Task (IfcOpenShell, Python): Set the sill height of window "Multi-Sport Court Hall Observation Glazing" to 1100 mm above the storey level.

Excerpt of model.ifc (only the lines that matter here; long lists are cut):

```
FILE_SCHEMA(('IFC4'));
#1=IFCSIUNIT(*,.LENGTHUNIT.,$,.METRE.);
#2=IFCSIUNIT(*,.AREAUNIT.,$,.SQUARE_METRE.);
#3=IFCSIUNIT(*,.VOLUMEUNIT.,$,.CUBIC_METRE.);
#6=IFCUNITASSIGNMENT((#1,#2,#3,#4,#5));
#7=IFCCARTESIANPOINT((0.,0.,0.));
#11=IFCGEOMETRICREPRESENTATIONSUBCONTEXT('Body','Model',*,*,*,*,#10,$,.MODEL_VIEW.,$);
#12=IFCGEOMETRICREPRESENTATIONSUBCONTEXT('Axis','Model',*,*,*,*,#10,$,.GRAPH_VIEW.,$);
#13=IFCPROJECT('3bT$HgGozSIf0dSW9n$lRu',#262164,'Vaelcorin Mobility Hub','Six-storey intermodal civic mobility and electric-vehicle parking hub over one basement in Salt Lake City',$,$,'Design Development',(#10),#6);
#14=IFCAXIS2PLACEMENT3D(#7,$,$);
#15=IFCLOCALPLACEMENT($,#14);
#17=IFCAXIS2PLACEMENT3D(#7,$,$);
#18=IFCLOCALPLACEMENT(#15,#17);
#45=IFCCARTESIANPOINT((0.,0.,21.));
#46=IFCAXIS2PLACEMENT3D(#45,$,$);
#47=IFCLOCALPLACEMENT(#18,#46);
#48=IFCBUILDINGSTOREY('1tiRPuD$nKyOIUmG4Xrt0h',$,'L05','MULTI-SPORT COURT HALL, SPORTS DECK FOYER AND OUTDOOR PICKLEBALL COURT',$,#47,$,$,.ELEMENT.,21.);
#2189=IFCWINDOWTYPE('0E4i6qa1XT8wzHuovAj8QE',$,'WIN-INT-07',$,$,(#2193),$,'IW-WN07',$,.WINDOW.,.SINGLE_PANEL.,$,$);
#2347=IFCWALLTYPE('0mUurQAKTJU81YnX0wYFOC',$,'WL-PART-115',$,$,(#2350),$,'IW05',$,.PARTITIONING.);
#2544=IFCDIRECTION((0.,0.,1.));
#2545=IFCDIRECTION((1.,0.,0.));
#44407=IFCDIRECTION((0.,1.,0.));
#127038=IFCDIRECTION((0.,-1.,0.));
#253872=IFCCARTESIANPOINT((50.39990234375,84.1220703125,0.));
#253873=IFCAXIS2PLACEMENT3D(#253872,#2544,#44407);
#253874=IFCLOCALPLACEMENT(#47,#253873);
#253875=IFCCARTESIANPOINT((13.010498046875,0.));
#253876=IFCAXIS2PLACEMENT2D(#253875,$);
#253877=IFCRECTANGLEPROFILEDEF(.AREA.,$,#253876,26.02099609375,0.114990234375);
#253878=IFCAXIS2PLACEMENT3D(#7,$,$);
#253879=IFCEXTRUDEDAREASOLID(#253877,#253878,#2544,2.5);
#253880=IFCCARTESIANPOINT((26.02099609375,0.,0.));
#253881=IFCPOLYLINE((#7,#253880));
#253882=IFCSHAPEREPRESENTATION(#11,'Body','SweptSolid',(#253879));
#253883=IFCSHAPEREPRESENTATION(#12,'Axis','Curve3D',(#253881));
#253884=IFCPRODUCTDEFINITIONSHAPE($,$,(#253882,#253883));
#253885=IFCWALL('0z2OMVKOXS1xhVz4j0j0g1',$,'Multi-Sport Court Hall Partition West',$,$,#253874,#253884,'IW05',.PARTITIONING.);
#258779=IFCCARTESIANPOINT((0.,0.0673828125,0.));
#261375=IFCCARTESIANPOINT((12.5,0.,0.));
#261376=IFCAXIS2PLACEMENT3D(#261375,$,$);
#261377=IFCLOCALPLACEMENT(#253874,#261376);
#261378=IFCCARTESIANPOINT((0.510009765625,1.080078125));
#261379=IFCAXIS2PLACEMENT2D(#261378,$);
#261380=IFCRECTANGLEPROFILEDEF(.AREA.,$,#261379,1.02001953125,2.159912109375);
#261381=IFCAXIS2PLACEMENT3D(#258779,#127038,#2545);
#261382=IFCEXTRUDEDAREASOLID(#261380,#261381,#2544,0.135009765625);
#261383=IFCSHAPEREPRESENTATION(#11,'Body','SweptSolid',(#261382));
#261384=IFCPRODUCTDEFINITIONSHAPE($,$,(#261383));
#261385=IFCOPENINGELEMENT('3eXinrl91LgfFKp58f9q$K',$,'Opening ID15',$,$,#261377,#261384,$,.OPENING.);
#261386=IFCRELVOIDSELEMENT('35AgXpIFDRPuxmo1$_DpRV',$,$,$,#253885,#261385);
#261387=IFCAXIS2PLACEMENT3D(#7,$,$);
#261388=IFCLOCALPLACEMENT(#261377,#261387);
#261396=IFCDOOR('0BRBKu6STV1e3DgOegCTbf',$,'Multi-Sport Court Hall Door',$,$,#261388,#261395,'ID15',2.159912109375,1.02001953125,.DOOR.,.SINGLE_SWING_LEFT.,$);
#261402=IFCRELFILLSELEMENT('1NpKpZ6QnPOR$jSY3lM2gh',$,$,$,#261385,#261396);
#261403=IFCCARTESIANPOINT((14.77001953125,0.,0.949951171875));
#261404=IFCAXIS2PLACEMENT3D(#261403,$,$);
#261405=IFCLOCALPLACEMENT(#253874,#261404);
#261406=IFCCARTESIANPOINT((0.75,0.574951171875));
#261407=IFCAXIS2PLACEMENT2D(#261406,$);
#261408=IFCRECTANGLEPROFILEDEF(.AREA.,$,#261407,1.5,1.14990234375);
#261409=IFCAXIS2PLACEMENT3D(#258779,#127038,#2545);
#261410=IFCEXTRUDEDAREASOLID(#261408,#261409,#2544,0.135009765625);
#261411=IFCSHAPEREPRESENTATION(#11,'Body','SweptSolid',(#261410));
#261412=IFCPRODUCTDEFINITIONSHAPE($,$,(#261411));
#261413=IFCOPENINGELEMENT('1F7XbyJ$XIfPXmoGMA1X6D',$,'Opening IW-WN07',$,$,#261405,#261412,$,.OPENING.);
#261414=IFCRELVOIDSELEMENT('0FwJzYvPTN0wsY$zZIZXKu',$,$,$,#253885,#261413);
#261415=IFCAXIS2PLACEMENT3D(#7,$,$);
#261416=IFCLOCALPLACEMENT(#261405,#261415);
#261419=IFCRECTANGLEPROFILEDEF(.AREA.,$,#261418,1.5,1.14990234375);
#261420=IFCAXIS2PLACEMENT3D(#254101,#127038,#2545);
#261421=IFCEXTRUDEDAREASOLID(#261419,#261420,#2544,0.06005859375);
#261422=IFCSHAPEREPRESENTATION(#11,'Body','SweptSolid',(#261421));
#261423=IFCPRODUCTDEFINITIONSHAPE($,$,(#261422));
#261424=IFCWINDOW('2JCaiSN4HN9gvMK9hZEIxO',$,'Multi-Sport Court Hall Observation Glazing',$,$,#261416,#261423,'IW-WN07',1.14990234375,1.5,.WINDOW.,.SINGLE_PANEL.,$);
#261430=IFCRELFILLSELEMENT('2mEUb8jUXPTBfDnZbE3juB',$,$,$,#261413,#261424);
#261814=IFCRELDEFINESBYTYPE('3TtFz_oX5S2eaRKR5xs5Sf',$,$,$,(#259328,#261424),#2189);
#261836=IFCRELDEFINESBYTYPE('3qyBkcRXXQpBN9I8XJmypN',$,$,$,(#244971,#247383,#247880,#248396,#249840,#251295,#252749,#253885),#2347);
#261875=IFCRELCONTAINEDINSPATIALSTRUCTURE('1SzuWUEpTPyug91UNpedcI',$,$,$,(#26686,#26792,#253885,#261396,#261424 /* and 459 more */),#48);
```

```python
import numpy as np
import ifcopenshell
import ifcopenshell.api.geometry
import ifcopenshell.geom
import ifcopenshell.util.element
import ifcopenshell.util.placement
import ifcopenshell.util.shape
import ifcopenshell.util.unit

model = ifcopenshell.open("model.ifc")
unit_scale = ifcopenshell.util.unit.calculate_unit_scale(model)

window = model.by_guid("2JCaiSN4HN9gvMK9hZEIxO")
opening = window.FillsVoids[0].RelatingOpeningElement
storey = ifcopenshell.util.element.get_container(window, ifc_class="IfcBuildingStorey")
level = ifcopenshell.util.placement.get_local_placement(storey.ObjectPlacement)[2, 3]

# The opening's origin need not be at the sill, so measure its lowest point.
shape = ifcopenshell.geom.create_shape(ifcopenshell.geom.settings(), opening)
bottom = ifcopenshell.util.shape.get_shape_bottom_elevation(shape, shape.geometry) / unit_scale
dz = level + 1.1 / unit_scale - bottom

shift = np.array([0.0, 0.0, dz])
# The window is placed relative to its opening, so it follows when the opening moves.
matrix = ifcopenshell.util.placement.get_local_placement(opening.ObjectPlacement)
matrix[:3, 3] += shift
ifcopenshell.api.geometry.edit_object_placement(
    model, product=opening, matrix=matrix, is_si=False, should_transform_children=True
)

print(f"moved by {dz * unit_scale:+.3f} m")

model.write("model_updated.ifc")
```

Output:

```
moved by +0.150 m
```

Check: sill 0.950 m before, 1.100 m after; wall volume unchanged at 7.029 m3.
